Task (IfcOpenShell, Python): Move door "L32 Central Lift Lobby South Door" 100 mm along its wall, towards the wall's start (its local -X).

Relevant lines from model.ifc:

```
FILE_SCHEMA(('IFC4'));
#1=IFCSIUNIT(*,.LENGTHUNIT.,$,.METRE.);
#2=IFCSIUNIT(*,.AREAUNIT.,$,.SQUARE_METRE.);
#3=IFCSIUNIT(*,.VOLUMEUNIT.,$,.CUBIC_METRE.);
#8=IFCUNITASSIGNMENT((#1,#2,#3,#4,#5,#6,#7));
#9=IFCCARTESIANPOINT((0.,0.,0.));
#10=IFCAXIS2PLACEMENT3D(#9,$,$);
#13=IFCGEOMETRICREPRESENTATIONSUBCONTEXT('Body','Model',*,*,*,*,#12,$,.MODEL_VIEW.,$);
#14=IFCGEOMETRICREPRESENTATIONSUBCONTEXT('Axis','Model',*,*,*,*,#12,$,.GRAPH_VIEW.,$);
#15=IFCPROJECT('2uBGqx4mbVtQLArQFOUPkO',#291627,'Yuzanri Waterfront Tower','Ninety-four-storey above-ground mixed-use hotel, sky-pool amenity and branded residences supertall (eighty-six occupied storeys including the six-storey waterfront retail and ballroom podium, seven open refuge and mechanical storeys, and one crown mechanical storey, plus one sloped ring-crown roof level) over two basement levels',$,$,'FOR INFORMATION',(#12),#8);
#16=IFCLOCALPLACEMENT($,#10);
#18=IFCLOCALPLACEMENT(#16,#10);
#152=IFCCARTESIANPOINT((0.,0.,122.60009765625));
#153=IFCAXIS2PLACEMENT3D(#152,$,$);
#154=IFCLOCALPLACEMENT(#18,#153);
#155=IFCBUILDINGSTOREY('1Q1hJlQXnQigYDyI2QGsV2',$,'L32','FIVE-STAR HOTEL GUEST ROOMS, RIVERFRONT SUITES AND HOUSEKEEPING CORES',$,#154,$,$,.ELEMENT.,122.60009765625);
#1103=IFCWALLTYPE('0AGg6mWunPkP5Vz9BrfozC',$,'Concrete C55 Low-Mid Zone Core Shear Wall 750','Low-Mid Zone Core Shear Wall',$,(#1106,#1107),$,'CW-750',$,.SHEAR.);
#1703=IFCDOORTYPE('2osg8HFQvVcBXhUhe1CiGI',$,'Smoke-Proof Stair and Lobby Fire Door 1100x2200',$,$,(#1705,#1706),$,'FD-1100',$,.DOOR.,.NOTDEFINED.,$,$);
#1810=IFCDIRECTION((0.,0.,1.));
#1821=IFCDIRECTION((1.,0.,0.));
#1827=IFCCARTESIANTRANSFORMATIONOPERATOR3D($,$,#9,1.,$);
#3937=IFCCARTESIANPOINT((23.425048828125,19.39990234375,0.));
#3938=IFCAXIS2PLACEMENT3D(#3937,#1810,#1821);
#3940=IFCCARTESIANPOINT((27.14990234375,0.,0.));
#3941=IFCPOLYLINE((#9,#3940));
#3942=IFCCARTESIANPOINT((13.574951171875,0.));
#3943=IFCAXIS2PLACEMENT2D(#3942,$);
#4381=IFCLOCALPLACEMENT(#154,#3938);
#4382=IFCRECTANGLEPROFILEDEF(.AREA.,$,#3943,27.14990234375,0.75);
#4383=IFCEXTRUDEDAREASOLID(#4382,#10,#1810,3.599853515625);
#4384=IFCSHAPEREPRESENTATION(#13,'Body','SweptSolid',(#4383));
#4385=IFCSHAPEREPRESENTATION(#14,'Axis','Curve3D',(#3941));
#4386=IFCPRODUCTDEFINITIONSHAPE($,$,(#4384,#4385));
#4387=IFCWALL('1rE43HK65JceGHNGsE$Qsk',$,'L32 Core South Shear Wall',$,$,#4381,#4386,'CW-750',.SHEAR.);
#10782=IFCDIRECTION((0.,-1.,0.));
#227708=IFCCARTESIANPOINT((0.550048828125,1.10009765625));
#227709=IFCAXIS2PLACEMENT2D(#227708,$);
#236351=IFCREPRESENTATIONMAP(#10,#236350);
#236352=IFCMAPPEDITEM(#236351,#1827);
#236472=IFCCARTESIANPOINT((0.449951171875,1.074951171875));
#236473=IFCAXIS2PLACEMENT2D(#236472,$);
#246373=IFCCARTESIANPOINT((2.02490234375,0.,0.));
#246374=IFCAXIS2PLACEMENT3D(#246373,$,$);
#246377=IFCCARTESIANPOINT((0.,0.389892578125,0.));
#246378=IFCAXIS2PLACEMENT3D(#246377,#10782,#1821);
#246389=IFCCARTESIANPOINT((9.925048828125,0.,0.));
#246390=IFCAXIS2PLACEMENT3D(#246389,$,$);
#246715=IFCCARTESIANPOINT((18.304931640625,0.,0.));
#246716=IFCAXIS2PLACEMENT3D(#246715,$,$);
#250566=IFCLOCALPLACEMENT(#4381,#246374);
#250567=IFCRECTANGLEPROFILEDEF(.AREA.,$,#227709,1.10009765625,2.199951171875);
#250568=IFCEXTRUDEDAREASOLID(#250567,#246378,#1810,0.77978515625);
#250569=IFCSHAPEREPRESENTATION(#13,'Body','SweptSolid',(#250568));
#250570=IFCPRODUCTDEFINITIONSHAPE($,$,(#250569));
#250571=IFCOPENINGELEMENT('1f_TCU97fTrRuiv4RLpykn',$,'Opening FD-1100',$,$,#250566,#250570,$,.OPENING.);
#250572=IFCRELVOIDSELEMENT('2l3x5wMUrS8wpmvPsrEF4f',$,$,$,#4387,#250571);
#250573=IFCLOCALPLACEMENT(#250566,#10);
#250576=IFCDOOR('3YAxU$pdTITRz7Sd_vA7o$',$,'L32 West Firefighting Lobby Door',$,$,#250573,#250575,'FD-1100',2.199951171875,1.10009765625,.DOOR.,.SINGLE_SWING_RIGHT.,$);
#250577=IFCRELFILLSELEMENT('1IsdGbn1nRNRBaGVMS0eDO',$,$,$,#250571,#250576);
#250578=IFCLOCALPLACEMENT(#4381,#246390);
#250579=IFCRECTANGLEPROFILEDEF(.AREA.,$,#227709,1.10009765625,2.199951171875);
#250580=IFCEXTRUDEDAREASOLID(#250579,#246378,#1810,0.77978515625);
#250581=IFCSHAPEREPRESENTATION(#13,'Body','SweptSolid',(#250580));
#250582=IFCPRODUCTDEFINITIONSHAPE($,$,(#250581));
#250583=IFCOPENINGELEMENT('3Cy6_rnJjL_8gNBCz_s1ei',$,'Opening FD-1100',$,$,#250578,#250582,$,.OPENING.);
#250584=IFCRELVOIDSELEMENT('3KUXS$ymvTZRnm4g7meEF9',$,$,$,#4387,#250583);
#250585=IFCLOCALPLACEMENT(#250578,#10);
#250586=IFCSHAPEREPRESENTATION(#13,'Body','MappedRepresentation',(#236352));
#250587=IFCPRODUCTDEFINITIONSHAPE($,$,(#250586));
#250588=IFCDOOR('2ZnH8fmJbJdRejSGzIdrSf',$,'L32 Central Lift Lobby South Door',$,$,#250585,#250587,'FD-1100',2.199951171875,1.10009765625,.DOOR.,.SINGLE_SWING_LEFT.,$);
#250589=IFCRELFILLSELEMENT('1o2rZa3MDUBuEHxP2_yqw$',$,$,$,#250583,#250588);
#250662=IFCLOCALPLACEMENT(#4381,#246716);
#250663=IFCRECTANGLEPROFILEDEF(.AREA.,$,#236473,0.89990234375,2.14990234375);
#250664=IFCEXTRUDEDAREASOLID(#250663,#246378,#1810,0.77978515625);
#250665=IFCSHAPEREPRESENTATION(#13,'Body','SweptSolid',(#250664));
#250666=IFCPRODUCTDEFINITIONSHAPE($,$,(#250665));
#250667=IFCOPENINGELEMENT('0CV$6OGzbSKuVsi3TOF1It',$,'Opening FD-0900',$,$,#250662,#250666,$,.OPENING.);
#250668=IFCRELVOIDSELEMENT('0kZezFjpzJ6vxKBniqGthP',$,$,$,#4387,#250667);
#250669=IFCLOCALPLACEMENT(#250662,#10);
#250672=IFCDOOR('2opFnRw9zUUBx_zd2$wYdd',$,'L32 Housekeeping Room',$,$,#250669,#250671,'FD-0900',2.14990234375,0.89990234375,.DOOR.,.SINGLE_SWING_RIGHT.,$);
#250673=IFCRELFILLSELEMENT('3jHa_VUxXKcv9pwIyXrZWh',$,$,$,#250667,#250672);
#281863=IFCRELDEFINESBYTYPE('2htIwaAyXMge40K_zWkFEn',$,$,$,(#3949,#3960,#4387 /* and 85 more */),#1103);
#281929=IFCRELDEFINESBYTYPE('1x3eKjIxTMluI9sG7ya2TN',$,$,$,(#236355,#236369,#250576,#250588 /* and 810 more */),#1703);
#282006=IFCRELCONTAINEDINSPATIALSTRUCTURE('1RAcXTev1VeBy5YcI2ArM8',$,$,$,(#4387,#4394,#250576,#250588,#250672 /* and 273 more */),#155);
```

```python
import ifcopenshell
import ifcopenshell.api.geometry
import ifcopenshell.util.placement
import ifcopenshell.util.unit

model = ifcopenshell.open("model.ifc")
unit_scale = ifcopenshell.util.unit.calculate_unit_scale(model)

door = model.by_guid("2ZnH8fmJbJdRejSGzIdrSf")
opening = door.FillsVoids[0].RelatingOpeningElement
wall = opening.VoidsElements[0].RelatingBuildingElement

wall_matrix = ifcopenshell.util.placement.get_local_placement(wall.ObjectPlacement)
shift = wall_matrix[:3, 0] * -0.1 / unit_scale
before = ifcopenshell.util.placement.get_local_placement(door.ObjectPlacement)[:3, 3].copy()

# The door is placed relative to its opening, so it follows when the opening moves.
matrix = ifcopenshell.util.placement.get_local_placement(opening.ObjectPlacement)
matrix[:3, 3] += shift
ifcopenshell.api.geometry.edit_object_placement(
    model, product=opening, matrix=matrix, is_si=False, should_transform_children=True
)

after = ifcopenshell.util.placement.get_local_placement(door.ObjectPlacement)[:3, 3]
print("door moved by", (after - before).round(3) + 0.0)

model.write("model_v2.ifc")
```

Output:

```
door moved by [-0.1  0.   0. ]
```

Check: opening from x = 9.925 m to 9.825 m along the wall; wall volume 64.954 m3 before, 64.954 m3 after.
